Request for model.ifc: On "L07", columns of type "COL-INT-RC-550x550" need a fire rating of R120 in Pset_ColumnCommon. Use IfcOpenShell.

First a look at what the model holds.

```python
import ifcopenshell
import ifcopenshell.util.element

model = ifcopenshell.open("model.ifc")
print(model.schema)
storey = next(s for s in model.by_type("IfcBuildingStorey") if s.Name == "L07")
columns = [e for e in ifcopenshell.util.element.get_decomposition(storey) if e.is_a("IfcColumn")]
seen = {}
for e in columns:
    element_type = ifcopenshell.util.element.get_type(e)
    key = (element_type.Name if element_type != e and element_type else None, ifcopenshell.util.element.get_pset(e, "Pset_ColumnCommon", "FireRating"))
    seen[key] = seen.get(key, 0) + 1
for (name, value), count in sorted(seen.items(), key=str):
    print(count, "x", name, "|", value)
```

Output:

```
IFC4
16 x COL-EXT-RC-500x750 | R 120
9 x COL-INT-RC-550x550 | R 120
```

```python
import ifcopenshell
import ifcopenshell.api.pset
import ifcopenshell.util.element

model = ifcopenshell.open("model.ifc")

storey = next(s for s in model.by_type("IfcBuildingStorey") if s.Name == "L07")
columns = [e for e in ifcopenshell.util.element.get_decomposition(storey) if e.is_a("IfcColumn")]

count = 0
for e in columns:
    element_type = ifcopenshell.util.element.get_type(e)
    if element_type in (None, e) or element_type.Name != "COL-INT-RC-550x550":
        continue
    # add_pset returns the element's existing set when there is one.
    pset = ifcopenshell.api.pset.add_pset(model, product=e, name="Pset_ColumnCommon")
    ifcopenshell.api.pset.edit_pset(model, pset=pset, properties={"FireRating": "R120"})
    count += 1

print(count, "columns updated")

model.write("model_rev.ifc")
```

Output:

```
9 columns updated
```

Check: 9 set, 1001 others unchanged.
